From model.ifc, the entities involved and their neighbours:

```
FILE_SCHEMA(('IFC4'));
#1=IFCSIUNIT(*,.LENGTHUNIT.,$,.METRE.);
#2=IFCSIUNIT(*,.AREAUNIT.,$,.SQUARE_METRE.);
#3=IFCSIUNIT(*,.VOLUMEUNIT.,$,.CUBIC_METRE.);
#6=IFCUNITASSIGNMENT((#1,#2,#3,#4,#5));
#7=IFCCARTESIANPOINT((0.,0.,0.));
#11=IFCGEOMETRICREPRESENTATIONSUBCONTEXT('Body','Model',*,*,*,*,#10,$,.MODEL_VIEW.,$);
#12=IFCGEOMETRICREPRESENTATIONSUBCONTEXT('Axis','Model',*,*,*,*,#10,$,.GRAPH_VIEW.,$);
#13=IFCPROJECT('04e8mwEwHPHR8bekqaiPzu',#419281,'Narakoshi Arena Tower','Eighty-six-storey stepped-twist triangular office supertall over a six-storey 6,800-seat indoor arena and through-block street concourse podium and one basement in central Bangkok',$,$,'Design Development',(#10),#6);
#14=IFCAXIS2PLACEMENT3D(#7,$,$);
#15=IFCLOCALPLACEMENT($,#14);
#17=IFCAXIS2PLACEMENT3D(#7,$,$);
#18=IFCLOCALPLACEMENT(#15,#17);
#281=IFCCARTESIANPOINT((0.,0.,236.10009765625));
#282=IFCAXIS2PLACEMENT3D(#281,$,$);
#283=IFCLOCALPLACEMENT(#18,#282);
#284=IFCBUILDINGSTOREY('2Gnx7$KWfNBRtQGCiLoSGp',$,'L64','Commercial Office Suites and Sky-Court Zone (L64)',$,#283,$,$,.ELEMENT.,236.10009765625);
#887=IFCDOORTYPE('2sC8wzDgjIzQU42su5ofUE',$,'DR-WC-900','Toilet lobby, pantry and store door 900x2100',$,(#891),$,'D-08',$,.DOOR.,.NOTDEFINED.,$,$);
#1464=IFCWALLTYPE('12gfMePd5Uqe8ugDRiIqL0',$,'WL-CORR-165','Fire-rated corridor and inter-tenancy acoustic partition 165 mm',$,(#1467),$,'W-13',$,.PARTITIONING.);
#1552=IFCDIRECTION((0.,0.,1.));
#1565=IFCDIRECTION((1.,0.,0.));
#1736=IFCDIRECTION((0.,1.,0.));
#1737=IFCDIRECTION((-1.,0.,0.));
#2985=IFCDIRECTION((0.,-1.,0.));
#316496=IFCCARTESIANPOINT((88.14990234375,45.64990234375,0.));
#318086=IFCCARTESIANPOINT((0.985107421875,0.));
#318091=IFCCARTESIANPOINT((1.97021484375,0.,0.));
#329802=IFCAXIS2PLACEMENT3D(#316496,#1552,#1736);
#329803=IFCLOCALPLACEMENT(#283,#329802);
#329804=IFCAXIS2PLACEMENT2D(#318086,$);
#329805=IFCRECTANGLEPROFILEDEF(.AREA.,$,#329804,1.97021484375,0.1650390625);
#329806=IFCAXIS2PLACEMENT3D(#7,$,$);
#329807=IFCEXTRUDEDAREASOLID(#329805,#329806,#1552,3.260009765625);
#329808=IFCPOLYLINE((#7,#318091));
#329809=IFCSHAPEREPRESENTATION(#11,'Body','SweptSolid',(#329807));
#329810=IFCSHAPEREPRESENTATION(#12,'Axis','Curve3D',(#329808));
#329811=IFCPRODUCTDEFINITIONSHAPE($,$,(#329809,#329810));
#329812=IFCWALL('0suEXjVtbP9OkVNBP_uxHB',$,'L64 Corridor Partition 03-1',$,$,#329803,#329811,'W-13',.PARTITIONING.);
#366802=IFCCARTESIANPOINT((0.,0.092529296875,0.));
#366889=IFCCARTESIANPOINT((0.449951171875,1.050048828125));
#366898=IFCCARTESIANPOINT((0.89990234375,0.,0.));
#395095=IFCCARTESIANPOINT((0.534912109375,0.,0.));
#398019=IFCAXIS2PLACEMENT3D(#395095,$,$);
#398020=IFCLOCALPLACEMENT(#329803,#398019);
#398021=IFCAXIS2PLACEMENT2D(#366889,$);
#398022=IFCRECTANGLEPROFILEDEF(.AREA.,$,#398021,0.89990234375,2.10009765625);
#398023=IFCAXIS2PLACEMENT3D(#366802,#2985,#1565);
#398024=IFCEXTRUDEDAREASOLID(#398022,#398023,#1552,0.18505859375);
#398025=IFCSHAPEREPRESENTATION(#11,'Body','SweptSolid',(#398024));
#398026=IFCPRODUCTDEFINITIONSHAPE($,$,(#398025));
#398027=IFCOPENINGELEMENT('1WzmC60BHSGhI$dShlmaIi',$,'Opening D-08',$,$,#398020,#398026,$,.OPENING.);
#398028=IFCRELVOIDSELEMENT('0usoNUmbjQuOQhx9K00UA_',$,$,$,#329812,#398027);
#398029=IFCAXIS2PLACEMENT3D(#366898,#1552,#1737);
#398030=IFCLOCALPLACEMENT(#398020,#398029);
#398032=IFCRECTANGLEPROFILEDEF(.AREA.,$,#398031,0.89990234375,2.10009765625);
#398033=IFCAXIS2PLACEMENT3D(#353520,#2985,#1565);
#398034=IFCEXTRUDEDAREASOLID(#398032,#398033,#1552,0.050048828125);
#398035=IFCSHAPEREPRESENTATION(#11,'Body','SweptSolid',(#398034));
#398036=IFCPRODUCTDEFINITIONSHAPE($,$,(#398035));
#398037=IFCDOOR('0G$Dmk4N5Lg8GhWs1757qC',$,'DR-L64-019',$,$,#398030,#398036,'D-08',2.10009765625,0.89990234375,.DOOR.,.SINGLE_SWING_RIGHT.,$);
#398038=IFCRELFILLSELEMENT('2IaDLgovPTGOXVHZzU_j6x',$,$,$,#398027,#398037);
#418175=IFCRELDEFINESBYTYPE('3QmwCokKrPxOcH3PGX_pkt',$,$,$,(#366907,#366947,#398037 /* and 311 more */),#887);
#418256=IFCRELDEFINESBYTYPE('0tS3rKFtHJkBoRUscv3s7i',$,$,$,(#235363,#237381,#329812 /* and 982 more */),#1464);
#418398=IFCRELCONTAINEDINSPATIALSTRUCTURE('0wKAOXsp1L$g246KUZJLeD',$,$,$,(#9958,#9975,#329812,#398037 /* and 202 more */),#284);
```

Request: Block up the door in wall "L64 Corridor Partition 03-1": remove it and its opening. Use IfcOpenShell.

```python
import ifcopenshell
import ifcopenshell.api.feature
import ifcopenshell.api.root
import ifcopenshell.geom
import ifcopenshell.util.shape

model = ifcopenshell.open("model.ifc")
settings = ifcopenshell.geom.settings()


def volume(element):
    """Net volume in cubic metres, openings subtracted."""
    shape = ifcopenshell.geom.create_shape(settings, element)
    return ifcopenshell.util.shape.get_volume(shape.geometry)


door = model.by_guid("0G$Dmk4N5Lg8GhWs1757qC")
opening = door.FillsVoids[0].RelatingOpeningElement
wall = opening.VoidsElements[0].RelatingBuildingElement
before = volume(wall)

ifcopenshell.api.root.remove_product(model, product=door)
ifcopenshell.api.feature.remove_feature(model, feature=opening)

after = volume(wall)

print(f"wall volume {before:.3f} -> {after:.3f} m3")

model.write("model_rev.ifc")
```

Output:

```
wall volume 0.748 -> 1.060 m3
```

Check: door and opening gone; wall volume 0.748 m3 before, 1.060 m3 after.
